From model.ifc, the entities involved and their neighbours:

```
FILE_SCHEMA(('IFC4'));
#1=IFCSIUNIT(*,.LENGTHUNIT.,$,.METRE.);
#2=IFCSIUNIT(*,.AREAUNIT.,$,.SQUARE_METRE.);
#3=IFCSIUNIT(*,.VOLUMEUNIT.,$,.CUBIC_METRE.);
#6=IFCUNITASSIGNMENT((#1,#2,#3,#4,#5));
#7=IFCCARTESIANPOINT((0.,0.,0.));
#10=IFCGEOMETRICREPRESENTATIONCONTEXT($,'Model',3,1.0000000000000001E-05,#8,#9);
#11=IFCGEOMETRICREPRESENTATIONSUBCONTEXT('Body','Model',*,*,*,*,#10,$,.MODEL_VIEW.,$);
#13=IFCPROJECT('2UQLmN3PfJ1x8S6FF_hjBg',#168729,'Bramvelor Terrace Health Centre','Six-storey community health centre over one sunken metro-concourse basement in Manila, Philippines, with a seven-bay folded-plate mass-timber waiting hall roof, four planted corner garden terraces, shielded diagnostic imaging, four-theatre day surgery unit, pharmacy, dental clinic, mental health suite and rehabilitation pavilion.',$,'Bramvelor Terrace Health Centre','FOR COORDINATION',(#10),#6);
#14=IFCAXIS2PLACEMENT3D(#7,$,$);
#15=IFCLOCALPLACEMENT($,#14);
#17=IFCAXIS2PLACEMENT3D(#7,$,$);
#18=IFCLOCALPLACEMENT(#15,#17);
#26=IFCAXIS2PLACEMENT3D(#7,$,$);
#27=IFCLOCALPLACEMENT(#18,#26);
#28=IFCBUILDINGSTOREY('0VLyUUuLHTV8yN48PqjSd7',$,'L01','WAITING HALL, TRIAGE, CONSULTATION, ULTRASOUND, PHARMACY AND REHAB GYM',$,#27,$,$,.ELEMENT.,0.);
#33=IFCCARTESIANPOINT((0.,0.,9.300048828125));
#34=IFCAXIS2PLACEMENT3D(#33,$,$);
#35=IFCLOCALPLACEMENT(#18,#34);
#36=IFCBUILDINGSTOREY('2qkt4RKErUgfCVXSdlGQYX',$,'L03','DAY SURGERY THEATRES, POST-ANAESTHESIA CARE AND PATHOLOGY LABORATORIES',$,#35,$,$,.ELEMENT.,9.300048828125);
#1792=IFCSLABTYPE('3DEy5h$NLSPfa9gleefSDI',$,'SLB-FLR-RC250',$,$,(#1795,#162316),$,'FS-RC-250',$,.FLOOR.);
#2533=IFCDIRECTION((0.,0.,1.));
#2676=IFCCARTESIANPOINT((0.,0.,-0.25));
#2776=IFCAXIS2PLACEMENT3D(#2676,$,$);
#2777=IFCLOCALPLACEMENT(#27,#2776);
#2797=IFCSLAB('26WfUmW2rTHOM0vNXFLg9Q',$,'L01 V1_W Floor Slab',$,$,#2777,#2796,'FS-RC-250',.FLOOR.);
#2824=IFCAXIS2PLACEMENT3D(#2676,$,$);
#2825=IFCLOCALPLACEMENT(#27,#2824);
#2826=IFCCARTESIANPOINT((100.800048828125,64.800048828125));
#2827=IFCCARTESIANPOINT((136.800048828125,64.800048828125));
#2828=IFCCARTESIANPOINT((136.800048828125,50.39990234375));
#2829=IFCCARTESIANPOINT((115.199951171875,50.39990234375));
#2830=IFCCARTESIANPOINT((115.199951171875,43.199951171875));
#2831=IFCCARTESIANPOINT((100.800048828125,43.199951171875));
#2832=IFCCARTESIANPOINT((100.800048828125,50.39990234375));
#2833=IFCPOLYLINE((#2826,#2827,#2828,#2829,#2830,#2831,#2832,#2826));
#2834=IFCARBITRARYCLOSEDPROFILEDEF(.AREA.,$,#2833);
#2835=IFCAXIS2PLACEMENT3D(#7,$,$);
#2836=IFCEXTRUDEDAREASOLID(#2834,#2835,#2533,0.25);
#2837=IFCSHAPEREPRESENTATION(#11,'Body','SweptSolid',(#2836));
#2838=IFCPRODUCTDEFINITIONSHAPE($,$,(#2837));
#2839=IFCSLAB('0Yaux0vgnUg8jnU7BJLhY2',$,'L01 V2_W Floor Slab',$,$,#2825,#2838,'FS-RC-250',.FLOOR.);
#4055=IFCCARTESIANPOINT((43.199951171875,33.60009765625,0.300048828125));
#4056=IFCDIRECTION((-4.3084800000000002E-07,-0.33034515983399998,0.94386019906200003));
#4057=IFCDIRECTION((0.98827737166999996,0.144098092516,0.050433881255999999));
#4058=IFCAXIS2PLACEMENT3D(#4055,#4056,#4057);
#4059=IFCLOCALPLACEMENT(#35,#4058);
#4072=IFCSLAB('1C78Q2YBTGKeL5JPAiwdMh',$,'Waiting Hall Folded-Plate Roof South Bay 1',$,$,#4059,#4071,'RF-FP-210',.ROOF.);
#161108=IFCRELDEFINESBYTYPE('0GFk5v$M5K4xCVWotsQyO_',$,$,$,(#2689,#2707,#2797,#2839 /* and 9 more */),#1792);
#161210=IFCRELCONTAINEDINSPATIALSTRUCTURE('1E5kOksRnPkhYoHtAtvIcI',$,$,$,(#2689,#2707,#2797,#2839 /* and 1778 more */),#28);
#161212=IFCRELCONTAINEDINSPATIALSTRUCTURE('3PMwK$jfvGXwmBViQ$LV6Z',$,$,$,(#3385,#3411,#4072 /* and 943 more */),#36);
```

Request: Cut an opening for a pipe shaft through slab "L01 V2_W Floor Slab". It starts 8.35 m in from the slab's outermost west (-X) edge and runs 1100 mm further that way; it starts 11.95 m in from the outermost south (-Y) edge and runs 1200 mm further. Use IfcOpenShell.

```python
import numpy as np
import ifcopenshell
import ifcopenshell.api.feature
import ifcopenshell.api.geometry
import ifcopenshell.api.root
import ifcopenshell.geom
import ifcopenshell.util.placement
import ifcopenshell.util.representation
import ifcopenshell.util.shape
import ifcopenshell.util.unit

model = ifcopenshell.open("model.ifc")
unit_scale = ifcopenshell.util.unit.calculate_unit_scale(model)
settings = ifcopenshell.geom.settings()


def volume(element):
    """Net volume in cubic metres, openings subtracted."""
    shape = ifcopenshell.geom.create_shape(settings, element)
    return ifcopenshell.util.shape.get_volume(shape.geometry)


slab = model.by_guid("0Yaux0vgnUg8jnU7BJLhY2")
before = volume(slab)

# Extent in the slab's own axes, in metres. The edges named are its -X and -Y sides.
slab_shape = ifcopenshell.geom.create_shape(settings, slab)
vertices = ifcopenshell.util.shape.get_vertices(slab_shape.geometry)
x_min, y_min, bottom = vertices.min(axis=0)
top = vertices[:, 2].max()

opening = ifcopenshell.api.root.create_entity(model, ifc_class="IfcOpeningElement", name="Pipe shaft opening", predefined_type="OPENING")
context = ifcopenshell.util.representation.get_context(model, "Model", "Body", "MODEL_VIEW")
width, depth = 1.1, 1.2
outline = [(0.0, 0.0), (width, 0.0), (width, depth), (0.0, depth), (0.0, 0.0)]
# Overshoot both faces by 50 mm so the cut is clean.
shape = ifcopenshell.api.geometry.add_slab_representation(
    model, context=context, depth=top - bottom + 0.1, polyline=outline
)
ifcopenshell.api.geometry.assign_representation(model, product=opening, representation=shape)

matrix = ifcopenshell.util.placement.get_local_placement(slab.ObjectPlacement)
matrix[:, 3] = matrix @ np.append(np.array([x_min + 8.35, y_min + 11.95, bottom - 0.05]) / unit_scale, 1.0)
ifcopenshell.api.geometry.edit_object_placement(model, product=opening, matrix=matrix, is_si=False)
ifcopenshell.api.feature.add_feature(model, feature=opening, element=slab)

after = volume(slab)

print(f"slab volume {before:.3f} -> {after:.3f} m3")

model.write("model_rev.ifc")
```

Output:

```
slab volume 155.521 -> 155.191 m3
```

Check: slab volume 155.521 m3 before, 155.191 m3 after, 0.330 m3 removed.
